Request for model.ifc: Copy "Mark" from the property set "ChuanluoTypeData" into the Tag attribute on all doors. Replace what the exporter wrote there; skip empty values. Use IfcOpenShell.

First a look at what the model holds.

```python
import ifcopenshell
import ifcopenshell.util.element

model = ifcopenshell.open("model.ifc")
print(model.schema)
doors = model.by_type("IfcDoor")
print(len(doors), "doors")
for e in doors[:8]:
    source = ifcopenshell.util.element.get_pset(e, "ChuanluoTypeData", "Mark")
    target = e.Tag
    print(e.id(), repr(source), repr(target), sep=" | ")
```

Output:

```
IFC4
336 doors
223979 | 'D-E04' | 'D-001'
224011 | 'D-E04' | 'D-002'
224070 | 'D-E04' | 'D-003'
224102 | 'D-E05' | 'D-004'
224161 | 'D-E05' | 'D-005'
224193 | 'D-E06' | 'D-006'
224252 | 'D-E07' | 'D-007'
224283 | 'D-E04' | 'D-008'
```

```python
import ifcopenshell
import ifcopenshell.util.element

model = ifcopenshell.open("model.ifc")

count = 0
for e in model.by_type("IfcDoor"):
    value = ifcopenshell.util.element.get_pset(e, "ChuanluoTypeData", "Mark")
    current = e.Tag
    if not value or not value.strip() or current == value:
        continue
    e.Tag = value
    count += 1

print(count, "doors updated")

model.write("model_rev.ifc")
```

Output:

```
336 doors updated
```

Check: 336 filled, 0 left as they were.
